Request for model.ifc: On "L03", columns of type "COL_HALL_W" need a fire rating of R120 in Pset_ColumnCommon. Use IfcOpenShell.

First a look at what the model holds.

```python
import ifcopenshell
import ifcopenshell.util.element

model = ifcopenshell.open("model.ifc")
print(model.schema)
storey = next(s for s in model.by_type("IfcBuildingStorey") if s.Name == "L03")
columns = [e for e in ifcopenshell.util.element.get_decomposition(storey) if e.is_a("IfcColumn")]
seen = {}
for e in columns:
    element_type = ifcopenshell.util.element.get_type(e)
    key = (element_type.Name if element_type != e and element_type else None, ifcopenshell.util.element.get_pset(e, "Pset_ColumnCommon", "FireRating"))
    seen[key] = seen.get(key, 0) + 1
for (name, value), count in sorted(seen.items(), key=str):
    print(count, "x", name, "|", value)
```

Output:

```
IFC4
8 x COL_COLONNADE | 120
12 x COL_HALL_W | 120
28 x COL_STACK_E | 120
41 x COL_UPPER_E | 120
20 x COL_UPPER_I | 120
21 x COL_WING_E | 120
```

```python
import ifcopenshell
import ifcopenshell.api.pset
import ifcopenshell.util.element

model = ifcopenshell.open("model.ifc")

storey = next(s for s in model.by_type("IfcBuildingStorey") if s.Name == "L03")
columns = [e for e in ifcopenshell.util.element.get_decomposition(storey) if e.is_a("IfcColumn")]

count = 0
for e in columns:
    element_type = ifcopenshell.util.element.get_type(e)
    if element_type in (None, e) or element_type.Name != "COL_HALL_W":
        continue
    # add_pset returns the element's existing set when there is one.
    pset = ifcopenshell.api.pset.add_pset(model, product=e, name="Pset_ColumnCommon")
    ifcopenshell.api.pset.edit_pset(model, pset=pset, properties={"FireRating": "R120"})
    count += 1

print(count, "columns updated")

model.write("model_rev.ifc")
```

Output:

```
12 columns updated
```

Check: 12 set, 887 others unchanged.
